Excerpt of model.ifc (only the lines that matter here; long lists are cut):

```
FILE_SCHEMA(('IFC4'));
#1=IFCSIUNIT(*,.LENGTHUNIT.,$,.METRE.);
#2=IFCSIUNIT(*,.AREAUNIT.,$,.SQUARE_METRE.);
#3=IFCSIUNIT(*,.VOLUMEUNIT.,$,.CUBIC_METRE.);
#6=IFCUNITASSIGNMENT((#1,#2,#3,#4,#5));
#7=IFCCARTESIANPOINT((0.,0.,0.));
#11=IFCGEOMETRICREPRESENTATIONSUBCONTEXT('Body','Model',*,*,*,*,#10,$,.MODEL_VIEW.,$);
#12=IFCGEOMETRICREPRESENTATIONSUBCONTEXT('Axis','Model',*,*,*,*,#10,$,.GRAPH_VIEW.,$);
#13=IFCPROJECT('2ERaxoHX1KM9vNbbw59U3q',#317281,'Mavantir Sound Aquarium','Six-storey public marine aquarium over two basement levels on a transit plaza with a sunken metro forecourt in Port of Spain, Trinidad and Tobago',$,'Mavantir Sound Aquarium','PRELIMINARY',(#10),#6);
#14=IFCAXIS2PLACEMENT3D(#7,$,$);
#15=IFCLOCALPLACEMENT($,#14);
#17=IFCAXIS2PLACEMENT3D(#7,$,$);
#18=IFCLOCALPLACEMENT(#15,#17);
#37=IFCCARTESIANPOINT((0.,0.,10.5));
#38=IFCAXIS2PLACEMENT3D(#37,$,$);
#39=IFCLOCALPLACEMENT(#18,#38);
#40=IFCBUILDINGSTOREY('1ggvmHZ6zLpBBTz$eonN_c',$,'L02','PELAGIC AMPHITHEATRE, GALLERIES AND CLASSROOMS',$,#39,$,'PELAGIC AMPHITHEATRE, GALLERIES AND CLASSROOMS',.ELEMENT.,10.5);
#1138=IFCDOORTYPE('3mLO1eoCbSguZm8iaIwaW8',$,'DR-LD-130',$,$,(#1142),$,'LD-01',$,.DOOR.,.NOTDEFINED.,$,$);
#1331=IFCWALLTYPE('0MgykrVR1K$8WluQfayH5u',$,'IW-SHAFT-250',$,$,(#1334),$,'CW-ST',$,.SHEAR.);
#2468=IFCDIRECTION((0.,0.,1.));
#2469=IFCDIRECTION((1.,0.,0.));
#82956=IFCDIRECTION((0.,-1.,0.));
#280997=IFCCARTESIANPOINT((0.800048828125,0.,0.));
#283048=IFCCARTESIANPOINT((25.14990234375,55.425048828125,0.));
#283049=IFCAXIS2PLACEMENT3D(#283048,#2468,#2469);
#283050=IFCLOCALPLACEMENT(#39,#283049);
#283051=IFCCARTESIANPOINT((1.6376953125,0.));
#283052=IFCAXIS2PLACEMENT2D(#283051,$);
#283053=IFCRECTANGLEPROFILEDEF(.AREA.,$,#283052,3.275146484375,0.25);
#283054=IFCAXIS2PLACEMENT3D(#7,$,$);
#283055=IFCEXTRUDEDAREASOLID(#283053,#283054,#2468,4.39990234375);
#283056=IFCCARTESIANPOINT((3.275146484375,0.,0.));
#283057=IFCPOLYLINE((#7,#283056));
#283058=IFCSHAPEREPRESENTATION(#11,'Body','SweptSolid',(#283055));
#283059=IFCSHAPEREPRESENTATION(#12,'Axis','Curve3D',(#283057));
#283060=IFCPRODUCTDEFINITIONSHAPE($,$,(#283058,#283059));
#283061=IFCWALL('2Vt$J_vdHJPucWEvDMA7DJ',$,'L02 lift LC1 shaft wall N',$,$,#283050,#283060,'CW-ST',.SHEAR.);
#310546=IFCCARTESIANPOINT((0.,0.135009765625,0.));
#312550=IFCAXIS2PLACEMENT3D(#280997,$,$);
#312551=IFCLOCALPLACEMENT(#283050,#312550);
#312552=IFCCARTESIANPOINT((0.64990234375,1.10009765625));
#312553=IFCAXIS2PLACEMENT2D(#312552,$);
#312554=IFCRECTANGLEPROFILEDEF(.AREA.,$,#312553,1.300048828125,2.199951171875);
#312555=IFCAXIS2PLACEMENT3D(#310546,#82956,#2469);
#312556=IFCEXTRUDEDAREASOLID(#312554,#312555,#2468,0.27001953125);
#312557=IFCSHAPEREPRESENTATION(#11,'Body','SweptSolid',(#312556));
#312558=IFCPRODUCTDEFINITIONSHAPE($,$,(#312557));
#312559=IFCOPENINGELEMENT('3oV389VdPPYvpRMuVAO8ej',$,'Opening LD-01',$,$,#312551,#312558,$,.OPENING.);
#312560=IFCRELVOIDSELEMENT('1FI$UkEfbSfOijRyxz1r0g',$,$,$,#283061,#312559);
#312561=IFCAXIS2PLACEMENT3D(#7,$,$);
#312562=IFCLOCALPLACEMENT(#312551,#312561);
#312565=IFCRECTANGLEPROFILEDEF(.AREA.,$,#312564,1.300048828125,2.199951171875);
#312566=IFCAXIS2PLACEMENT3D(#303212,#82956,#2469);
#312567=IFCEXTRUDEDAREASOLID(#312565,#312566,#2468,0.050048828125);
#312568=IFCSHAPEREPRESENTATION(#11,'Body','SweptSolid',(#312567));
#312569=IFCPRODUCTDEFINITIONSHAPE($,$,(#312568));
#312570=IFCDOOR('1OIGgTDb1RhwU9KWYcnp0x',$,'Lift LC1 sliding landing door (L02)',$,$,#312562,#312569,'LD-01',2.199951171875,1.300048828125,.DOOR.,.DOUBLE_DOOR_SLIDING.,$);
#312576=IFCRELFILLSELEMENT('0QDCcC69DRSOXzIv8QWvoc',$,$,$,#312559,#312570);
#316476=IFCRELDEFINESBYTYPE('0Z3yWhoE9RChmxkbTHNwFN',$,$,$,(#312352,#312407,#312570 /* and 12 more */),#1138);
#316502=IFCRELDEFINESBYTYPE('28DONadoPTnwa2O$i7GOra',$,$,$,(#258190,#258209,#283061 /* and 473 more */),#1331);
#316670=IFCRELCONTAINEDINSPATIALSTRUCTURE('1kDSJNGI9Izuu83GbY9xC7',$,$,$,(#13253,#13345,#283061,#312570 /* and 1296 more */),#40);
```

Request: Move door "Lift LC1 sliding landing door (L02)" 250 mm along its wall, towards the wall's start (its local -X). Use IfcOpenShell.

```python
import ifcopenshell
import ifcopenshell.api.geometry
import ifcopenshell.util.placement
import ifcopenshell.util.unit

model = ifcopenshell.open("model.ifc")
unit_scale = ifcopenshell.util.unit.calculate_unit_scale(model)

door = model.by_id(312570)
opening = door.FillsVoids[0].RelatingOpeningElement
wall = opening.VoidsElements[0].RelatingBuildingElement

wall_matrix = ifcopenshell.util.placement.get_local_placement(wall.ObjectPlacement)
shift = wall_matrix[:3, 0] * -0.25 / unit_scale
before = ifcopenshell.util.placement.get_local_placement(door.ObjectPlacement)[:3, 3].copy()

# The door is placed relative to its opening, so it follows when the opening moves.
matrix = ifcopenshell.util.placement.get_local_placement(opening.ObjectPlacement)
matrix[:3, 3] += shift
ifcopenshell.api.geometry.edit_object_placement(
    model, product=opening, matrix=matrix, is_si=False, should_transform_children=True
)

after = ifcopenshell.util.placement.get_local_placement(door.ObjectPlacement)[:3, 3]
print("door moved by", (after - before).round(3) + 0.0)

model.write("model_rev.ifc")
```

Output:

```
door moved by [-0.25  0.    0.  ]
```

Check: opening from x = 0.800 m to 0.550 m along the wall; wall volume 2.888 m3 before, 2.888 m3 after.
